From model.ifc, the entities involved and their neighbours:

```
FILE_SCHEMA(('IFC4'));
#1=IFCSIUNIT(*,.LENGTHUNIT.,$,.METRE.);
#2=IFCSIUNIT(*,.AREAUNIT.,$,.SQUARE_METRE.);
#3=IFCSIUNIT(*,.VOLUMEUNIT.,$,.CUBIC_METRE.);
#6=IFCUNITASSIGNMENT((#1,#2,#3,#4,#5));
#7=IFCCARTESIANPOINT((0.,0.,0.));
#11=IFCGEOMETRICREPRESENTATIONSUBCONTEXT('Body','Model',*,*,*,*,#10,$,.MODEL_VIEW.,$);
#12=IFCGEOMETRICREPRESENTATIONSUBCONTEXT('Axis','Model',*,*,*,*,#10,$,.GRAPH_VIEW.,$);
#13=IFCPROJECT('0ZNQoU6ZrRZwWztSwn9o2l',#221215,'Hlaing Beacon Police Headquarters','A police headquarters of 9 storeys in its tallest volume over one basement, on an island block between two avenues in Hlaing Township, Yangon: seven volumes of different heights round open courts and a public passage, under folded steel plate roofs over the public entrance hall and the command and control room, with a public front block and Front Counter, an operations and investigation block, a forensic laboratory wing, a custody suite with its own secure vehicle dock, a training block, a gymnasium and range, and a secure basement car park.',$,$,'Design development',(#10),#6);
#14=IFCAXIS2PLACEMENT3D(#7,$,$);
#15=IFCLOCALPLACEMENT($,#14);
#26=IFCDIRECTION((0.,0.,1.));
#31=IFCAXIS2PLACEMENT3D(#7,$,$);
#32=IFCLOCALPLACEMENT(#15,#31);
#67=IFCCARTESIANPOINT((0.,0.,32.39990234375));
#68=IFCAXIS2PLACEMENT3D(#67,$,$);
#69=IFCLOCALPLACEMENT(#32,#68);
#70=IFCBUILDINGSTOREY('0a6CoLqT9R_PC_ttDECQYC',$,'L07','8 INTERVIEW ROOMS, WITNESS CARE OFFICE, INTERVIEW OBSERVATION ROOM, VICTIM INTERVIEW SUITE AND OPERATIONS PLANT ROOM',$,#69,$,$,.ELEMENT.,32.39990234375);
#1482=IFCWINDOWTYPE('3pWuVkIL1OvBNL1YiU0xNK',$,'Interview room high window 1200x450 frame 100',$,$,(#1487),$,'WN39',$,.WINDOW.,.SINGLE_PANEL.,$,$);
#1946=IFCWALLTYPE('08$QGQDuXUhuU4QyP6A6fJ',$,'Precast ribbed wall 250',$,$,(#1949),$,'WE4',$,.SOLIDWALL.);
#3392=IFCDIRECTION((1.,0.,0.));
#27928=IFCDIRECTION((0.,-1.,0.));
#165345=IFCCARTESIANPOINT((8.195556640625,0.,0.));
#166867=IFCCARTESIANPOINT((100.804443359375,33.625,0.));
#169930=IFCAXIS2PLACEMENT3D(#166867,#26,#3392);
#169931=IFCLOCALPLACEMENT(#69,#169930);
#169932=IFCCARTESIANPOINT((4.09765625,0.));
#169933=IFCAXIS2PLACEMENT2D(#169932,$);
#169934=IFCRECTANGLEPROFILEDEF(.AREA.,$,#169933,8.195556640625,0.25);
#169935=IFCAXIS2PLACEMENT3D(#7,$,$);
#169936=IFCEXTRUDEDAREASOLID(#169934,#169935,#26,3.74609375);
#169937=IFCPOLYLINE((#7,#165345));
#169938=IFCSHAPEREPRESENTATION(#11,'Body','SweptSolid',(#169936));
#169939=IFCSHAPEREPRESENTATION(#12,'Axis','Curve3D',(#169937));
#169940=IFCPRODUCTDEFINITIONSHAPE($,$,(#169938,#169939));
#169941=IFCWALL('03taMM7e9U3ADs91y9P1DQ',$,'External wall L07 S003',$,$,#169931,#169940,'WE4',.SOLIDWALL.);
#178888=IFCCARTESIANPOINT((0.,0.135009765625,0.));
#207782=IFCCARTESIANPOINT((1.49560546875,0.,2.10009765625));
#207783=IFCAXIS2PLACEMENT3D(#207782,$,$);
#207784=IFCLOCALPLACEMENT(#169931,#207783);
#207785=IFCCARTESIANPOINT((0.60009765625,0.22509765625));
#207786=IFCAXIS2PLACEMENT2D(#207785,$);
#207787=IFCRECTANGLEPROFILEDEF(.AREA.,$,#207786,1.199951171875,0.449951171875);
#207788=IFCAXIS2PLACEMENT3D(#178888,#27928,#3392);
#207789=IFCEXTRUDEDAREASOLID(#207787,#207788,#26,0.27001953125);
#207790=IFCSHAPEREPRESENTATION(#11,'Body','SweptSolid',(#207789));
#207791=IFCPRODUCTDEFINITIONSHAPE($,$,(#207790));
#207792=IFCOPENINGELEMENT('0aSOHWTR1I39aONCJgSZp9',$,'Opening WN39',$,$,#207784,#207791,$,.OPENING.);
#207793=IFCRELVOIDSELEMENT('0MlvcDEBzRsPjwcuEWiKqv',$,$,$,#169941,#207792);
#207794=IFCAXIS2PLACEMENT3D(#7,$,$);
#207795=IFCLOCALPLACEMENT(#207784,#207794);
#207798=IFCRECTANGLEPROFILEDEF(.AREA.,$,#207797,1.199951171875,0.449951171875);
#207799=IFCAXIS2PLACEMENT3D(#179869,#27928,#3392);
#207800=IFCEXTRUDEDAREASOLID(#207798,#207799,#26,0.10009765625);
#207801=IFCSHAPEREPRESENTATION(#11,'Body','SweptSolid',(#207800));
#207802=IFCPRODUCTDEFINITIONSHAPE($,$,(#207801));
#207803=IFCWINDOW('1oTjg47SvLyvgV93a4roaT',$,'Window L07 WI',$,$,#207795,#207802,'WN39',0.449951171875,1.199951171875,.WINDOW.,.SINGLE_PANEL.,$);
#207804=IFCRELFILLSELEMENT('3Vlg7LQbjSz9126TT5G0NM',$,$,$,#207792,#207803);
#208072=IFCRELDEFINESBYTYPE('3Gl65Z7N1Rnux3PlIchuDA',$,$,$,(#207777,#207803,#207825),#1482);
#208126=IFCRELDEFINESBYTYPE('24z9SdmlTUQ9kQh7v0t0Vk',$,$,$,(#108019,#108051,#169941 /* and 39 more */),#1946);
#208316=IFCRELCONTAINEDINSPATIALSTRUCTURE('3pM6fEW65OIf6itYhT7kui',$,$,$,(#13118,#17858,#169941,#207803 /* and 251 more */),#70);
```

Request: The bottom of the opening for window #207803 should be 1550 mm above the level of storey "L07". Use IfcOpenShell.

```python
import numpy as np
import ifcopenshell
import ifcopenshell.api.geometry
import ifcopenshell.geom
import ifcopenshell.util.element
import ifcopenshell.util.placement
import ifcopenshell.util.shape
import ifcopenshell.util.unit

model = ifcopenshell.open("model.ifc")
unit_scale = ifcopenshell.util.unit.calculate_unit_scale(model)

window = model.by_id(207803)
opening = window.FillsVoids[0].RelatingOpeningElement
storey = ifcopenshell.util.element.get_container(window, ifc_class="IfcBuildingStorey")
level = ifcopenshell.util.placement.get_local_placement(storey.ObjectPlacement)[2, 3]

# The opening's origin need not be at the sill, so measure its lowest point.
shape = ifcopenshell.geom.create_shape(ifcopenshell.geom.settings(), opening)
bottom = ifcopenshell.util.shape.get_shape_bottom_elevation(shape, shape.geometry) / unit_scale
dz = level + 1.55 / unit_scale - bottom

shift = np.array([0.0, 0.0, dz])
# The window is placed relative to its opening, so it follows when the opening moves.
matrix = ifcopenshell.util.placement.get_local_placement(opening.ObjectPlacement)
matrix[:3, 3] += shift
ifcopenshell.api.geometry.edit_object_placement(
    model, product=opening, matrix=matrix, is_si=False, should_transform_children=True
)

print(f"moved by {dz * unit_scale:+.3f} m")

model.write("model_rev.ifc")
```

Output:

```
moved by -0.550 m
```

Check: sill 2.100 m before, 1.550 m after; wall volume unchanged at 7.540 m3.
